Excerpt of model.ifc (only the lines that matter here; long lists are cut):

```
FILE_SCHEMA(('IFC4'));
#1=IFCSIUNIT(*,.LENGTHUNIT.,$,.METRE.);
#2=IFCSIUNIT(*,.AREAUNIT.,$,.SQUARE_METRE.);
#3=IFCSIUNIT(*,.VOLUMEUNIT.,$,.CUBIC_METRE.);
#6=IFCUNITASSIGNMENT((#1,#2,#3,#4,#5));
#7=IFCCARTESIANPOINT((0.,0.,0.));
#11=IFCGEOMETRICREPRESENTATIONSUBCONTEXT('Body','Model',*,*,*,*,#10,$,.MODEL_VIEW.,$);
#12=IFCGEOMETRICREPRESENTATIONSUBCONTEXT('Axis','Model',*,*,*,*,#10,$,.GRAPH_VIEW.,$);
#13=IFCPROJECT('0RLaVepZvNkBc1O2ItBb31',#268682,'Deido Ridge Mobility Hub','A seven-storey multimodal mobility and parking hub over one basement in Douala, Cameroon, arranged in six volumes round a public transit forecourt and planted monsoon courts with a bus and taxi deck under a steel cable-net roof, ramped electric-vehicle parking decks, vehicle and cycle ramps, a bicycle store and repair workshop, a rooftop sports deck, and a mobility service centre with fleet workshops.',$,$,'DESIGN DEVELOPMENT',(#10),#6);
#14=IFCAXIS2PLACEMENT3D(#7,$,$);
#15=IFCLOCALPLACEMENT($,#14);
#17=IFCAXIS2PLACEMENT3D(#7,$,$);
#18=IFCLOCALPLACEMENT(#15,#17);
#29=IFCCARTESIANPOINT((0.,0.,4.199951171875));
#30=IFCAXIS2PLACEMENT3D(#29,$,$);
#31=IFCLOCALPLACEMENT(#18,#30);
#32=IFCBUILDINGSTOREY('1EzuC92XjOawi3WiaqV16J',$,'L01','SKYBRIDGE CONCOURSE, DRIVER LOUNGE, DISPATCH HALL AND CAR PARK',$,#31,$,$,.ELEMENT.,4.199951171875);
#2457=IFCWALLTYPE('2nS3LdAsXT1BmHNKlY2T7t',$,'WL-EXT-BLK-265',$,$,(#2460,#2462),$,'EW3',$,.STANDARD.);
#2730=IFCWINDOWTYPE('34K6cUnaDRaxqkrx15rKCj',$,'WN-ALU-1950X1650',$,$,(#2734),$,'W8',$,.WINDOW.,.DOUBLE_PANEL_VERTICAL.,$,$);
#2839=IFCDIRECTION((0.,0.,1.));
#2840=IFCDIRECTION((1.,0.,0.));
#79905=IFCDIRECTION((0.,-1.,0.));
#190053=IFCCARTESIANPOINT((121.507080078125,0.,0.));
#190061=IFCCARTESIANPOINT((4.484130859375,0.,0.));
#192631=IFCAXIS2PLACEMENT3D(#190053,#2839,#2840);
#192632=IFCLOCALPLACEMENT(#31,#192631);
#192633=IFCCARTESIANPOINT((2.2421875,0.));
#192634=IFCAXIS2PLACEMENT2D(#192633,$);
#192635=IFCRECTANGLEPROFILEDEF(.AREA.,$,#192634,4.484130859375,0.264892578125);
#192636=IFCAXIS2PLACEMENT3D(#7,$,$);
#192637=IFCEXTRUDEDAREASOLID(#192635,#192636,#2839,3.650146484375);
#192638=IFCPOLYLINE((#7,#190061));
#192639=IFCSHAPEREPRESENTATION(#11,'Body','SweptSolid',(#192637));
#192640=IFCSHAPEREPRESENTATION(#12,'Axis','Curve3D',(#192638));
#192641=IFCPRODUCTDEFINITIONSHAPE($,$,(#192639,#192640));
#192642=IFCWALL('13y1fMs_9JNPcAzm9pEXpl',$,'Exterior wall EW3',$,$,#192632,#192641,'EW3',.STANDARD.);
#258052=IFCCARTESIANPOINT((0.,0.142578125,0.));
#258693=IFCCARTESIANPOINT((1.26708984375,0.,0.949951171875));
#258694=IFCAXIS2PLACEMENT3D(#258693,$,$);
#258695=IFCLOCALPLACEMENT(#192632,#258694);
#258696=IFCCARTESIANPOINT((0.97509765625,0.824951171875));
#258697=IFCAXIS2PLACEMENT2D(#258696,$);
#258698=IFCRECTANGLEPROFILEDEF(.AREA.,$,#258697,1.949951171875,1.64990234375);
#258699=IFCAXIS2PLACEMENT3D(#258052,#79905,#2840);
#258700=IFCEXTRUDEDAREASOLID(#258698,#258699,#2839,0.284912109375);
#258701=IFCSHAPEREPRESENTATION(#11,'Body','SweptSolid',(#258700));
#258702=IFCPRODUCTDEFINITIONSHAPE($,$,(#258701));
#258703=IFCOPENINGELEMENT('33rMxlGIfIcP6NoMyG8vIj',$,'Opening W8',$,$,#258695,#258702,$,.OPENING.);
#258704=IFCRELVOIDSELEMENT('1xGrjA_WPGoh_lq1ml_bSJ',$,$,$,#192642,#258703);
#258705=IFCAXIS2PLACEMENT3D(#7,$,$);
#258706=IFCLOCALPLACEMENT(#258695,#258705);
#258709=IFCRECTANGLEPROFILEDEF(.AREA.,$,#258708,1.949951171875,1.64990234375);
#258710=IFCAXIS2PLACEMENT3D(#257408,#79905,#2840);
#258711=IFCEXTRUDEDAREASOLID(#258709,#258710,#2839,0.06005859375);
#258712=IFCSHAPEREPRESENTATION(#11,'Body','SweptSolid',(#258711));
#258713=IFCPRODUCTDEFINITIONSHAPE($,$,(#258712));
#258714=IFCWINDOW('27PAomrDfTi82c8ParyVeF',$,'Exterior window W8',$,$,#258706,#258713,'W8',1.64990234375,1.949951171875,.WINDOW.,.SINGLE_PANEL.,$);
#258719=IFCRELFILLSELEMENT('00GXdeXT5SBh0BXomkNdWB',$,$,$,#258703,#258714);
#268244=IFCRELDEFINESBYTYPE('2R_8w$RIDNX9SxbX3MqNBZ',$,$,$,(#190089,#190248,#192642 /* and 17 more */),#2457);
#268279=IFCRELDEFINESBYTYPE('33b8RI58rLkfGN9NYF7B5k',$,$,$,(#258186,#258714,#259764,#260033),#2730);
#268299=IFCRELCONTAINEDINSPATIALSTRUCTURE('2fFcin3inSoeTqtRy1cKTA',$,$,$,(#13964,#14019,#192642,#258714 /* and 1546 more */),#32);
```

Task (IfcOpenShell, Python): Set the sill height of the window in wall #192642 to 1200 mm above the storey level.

```python
import numpy as np
import ifcopenshell
import ifcopenshell.api.geometry
import ifcopenshell.geom
import ifcopenshell.util.element
import ifcopenshell.util.placement
import ifcopenshell.util.shape
import ifcopenshell.util.unit

model = ifcopenshell.open("model.ifc")
unit_scale = ifcopenshell.util.unit.calculate_unit_scale(model)

window = model.by_guid("27PAomrDfTi82c8ParyVeF")
opening = window.FillsVoids[0].RelatingOpeningElement
storey = ifcopenshell.util.element.get_container(window, ifc_class="IfcBuildingStorey")
level = ifcopenshell.util.placement.get_local_placement(storey.ObjectPlacement)[2, 3]

# The opening's origin need not be at the sill, so measure its lowest point.
shape = ifcopenshell.geom.create_shape(ifcopenshell.geom.settings(), opening)
bottom = ifcopenshell.util.shape.get_shape_bottom_elevation(shape, shape.geometry) / unit_scale
dz = level + 1.2 - bottom

shift = np.array([0.0, 0.0, dz])
# The window is placed relative to its opening, so it follows when the opening moves.
matrix = ifcopenshell.util.placement.get_local_placement(opening.ObjectPlacement)
matrix[:3, 3] += shift
ifcopenshell.api.geometry.edit_object_placement(
    model, product=opening, matrix=matrix, is_si=False, should_transform_children=True
)

print(f"moved by {dz * unit_scale:+.3f} m")

model.write("model_v2.ifc")
```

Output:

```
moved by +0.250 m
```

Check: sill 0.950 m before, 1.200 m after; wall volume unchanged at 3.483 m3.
